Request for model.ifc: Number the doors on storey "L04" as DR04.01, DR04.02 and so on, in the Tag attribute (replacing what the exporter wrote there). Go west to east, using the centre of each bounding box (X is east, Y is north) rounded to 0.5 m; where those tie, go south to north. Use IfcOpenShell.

First a look at what the model holds.

```python
import ifcopenshell
import ifcopenshell.util.element
import ifcopenshell.util.placement

model = ifcopenshell.open("model.ifc")
print(model.schema)
storey = next(s for s in model.by_type("IfcBuildingStorey") if s.Name == "L04")
doors = [e for e in ifcopenshell.util.element.get_decomposition(storey) if e.is_a("IfcDoor")]
for e in sorted(doors, key=lambda e: e.id()):
    origin = ifcopenshell.util.placement.get_local_placement(e.ObjectPlacement)[:3, 3]
    print(e.id(), e.Tag, e.Name, origin.round(2) + 0.0, sep=" | ")
```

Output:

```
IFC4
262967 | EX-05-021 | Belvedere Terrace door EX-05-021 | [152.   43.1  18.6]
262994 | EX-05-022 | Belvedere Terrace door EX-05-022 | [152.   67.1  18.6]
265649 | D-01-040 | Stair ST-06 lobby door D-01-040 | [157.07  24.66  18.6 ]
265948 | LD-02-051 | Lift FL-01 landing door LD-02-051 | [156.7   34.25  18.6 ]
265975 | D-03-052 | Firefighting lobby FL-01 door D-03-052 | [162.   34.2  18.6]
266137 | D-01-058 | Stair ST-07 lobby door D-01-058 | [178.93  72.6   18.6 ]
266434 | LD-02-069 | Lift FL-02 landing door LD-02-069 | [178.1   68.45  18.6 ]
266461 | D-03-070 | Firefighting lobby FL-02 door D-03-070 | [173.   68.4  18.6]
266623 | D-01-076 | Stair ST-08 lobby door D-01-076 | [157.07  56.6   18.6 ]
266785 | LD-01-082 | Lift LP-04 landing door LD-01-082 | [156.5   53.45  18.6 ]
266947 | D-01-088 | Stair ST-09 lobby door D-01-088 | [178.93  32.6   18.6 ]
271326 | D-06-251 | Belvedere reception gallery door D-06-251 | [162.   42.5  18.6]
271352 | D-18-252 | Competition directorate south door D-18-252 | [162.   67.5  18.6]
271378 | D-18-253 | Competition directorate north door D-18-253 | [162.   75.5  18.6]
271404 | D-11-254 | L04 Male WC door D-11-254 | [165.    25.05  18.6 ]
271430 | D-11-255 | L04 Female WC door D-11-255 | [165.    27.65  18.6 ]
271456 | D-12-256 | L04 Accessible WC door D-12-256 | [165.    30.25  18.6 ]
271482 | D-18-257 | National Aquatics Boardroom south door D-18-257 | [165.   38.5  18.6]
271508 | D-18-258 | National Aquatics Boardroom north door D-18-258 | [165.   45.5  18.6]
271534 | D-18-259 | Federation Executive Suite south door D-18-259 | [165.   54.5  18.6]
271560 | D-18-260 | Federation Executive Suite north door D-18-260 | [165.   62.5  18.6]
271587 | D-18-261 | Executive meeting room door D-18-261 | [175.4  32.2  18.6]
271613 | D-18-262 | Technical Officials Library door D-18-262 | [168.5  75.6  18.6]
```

```python
import ifcopenshell
import ifcopenshell.geom
import ifcopenshell.util.element
import ifcopenshell.util.shape

model = ifcopenshell.open("model.ifc")
settings = ifcopenshell.geom.settings()
settings.set("use-world-coords", True)


def centre(element):
    shape = ifcopenshell.geom.create_shape(settings, element)
    return ifcopenshell.util.shape.get_bbox_centroid(shape.geometry)


storey = next(s for s in model.by_type("IfcBuildingStorey") if s.Name == "L04")
doors = [e for e in ifcopenshell.util.element.get_decomposition(storey) if e.is_a("IfcDoor")]

# Insertion points can sit at a corner or the storey origin, so sort by the geometry (in metres).
centres = {e: centre(e) for e in doors}
doors.sort(key=lambda e: (round(centres[e][0] / 0.5), centres[e][1]))

for i, e in enumerate(doors, start=1):
    number = f"DR04.{i:02d}"
    e.Tag = number
    print(e.id(), number)

model.write("model_rev.ifc")
```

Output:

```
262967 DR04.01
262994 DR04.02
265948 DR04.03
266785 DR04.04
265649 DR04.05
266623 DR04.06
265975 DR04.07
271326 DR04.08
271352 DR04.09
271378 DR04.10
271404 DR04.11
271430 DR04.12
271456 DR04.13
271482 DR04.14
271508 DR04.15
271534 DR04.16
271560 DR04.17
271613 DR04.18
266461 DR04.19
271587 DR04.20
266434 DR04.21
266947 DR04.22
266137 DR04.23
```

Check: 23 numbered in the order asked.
